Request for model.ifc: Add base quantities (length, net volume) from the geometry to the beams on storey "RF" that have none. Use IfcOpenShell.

First a look at what the model holds.

```python
import ifcopenshell
import ifcopenshell.util.element
import ifcopenshell.util.unit

model = ifcopenshell.open("model.ifc")
print(model.schema)
for unit_type in ("LENGTHUNIT", "AREAUNIT", "VOLUMEUNIT"):
    print(unit_type, ifcopenshell.util.unit.calculate_unit_scale(model, unit_type))
storey = next(s for s in model.by_type("IfcBuildingStorey") if s.Name == "RF")
beams = [e for e in ifcopenshell.util.element.get_decomposition(storey) if e.is_a("IfcBeam")]
for e in sorted(beams, key=lambda e: e.id()):
    print(e.id(), e.is_a(), e.Name, list(ifcopenshell.util.element.get_psets(e, qtos_only=True)), sep=" | ")
```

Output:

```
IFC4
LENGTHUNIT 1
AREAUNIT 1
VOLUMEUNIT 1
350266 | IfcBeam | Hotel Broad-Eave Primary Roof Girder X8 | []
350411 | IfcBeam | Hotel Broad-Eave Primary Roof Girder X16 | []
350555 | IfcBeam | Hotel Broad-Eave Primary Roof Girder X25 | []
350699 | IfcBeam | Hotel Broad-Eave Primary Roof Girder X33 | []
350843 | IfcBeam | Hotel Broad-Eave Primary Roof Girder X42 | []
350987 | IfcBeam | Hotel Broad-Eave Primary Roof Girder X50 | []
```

```python
import ifcopenshell
import ifcopenshell.api.pset
import ifcopenshell.geom
import ifcopenshell.util.element
import ifcopenshell.util.shape
import ifcopenshell.util.unit

model = ifcopenshell.open("model.ifc")
unit_scale = ifcopenshell.util.unit.calculate_unit_scale(model)
volume_scale = ifcopenshell.util.unit.calculate_unit_scale(model, "VOLUMEUNIT")
settings = ifcopenshell.geom.settings()

storey = next(s for s in model.by_type("IfcBuildingStorey") if s.Name == "RF")
beams = [e for e in ifcopenshell.util.element.get_decomposition(storey) if e.is_a("IfcBeam")]

for e in sorted(beams, key=lambda e: e.id()):
    if ifcopenshell.util.element.get_psets(e, qtos_only=True, should_inherit=False):
        continue
    # Geometry comes back in metres, in the element's own axes.
    shape = ifcopenshell.geom.create_shape(settings, e)
    values = {
        "Length": ifcopenshell.util.shape.get_max_xyz(shape.geometry) / unit_scale,
        "NetVolume": ifcopenshell.util.shape.get_volume(shape.geometry) / volume_scale,
    }
    qto = ifcopenshell.api.pset.add_qto(model, product=e, name="Qto_BeamBaseQuantities")
    ifcopenshell.api.pset.edit_qto(model, qto=qto, properties=values)
    print(e.id(), {k: round(v, 3) for k, v in values.items()})

model.write("model_edited.ifc")
```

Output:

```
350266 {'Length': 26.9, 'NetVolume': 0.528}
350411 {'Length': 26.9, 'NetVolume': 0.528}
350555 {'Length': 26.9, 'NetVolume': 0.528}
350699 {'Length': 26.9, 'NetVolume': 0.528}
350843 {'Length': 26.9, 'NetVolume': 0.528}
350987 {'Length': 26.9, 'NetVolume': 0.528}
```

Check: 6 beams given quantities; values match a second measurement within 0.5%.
